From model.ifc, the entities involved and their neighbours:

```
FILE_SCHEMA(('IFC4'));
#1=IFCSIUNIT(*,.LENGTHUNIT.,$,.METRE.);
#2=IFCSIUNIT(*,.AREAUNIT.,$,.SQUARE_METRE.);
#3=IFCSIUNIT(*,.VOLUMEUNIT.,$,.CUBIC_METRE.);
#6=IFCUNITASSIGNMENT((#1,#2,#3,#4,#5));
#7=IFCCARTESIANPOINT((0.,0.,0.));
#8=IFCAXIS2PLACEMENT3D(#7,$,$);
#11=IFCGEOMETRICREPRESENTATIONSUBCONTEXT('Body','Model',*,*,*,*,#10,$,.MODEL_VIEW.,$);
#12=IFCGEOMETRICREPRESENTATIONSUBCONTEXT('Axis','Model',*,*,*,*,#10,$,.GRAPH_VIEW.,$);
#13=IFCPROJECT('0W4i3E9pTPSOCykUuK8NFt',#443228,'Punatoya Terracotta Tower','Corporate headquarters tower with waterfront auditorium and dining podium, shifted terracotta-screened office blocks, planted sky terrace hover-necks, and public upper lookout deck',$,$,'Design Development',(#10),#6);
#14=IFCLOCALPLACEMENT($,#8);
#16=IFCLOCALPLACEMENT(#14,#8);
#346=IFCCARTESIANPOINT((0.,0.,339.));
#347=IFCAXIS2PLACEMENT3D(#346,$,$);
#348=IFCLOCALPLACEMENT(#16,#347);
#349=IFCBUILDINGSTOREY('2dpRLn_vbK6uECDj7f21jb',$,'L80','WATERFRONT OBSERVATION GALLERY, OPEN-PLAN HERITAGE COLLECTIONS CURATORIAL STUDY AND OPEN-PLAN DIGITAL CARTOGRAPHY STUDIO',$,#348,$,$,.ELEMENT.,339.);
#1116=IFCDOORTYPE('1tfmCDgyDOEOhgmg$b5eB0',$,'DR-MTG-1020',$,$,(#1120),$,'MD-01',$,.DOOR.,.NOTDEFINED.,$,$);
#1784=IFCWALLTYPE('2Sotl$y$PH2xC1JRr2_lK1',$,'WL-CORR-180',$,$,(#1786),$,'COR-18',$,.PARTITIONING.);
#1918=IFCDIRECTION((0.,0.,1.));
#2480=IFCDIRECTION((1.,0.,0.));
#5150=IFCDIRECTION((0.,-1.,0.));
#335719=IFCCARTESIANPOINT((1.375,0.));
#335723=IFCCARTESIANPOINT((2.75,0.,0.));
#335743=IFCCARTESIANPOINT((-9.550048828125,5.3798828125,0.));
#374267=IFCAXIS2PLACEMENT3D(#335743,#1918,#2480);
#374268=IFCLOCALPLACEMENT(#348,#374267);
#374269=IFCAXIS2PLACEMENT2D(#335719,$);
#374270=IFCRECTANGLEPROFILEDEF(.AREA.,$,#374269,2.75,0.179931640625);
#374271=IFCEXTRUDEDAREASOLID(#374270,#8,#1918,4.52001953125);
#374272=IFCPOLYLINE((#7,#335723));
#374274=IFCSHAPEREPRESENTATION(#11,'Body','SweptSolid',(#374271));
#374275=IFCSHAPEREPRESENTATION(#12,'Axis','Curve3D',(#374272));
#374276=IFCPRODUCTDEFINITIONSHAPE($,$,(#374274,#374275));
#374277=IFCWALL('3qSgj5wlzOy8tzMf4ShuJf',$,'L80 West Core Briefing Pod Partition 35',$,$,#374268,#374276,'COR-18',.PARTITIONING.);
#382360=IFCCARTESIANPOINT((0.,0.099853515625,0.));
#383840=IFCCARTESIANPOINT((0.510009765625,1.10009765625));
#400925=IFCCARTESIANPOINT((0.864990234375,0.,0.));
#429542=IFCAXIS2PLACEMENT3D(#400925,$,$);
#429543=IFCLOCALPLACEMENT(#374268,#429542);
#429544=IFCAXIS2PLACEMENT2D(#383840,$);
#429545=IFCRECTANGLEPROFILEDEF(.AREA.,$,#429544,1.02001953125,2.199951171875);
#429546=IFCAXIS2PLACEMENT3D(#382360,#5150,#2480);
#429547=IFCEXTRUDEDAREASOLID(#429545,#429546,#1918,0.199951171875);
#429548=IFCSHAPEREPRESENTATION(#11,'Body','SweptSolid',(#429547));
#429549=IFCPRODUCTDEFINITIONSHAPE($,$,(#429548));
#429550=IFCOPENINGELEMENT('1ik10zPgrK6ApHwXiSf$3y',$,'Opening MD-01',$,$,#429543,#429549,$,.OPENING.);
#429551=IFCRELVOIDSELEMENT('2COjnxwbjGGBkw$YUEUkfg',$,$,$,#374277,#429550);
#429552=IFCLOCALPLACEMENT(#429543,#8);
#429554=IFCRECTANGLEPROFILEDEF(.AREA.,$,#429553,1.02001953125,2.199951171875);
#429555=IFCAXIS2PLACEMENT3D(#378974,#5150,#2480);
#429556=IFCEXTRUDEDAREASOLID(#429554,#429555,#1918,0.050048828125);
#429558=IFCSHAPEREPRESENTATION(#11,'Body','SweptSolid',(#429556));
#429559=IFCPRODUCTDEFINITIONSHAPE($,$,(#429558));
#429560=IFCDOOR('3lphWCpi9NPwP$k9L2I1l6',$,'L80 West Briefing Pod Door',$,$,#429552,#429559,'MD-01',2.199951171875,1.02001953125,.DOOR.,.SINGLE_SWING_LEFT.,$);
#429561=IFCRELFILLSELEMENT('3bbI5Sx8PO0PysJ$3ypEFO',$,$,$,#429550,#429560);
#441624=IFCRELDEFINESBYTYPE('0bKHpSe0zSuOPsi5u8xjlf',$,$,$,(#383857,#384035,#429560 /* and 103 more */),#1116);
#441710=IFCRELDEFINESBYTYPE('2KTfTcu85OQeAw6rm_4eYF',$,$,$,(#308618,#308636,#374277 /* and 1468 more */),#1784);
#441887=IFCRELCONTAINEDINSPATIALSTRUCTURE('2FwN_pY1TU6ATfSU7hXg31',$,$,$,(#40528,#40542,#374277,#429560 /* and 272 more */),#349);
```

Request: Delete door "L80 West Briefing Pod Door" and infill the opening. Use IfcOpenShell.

```python
import ifcopenshell
import ifcopenshell.api.feature
import ifcopenshell.api.root
import ifcopenshell.geom
import ifcopenshell.util.shape

model = ifcopenshell.open("model.ifc")
settings = ifcopenshell.geom.settings()


def volume(element):
    """Net volume in cubic metres, openings subtracted."""
    shape = ifcopenshell.geom.create_shape(settings, element)
    return ifcopenshell.util.shape.get_volume(shape.geometry)


door = model.by_guid("3lphWCpi9NPwP$k9L2I1l6")
opening = door.FillsVoids[0].RelatingOpeningElement
wall = opening.VoidsElements[0].RelatingBuildingElement
before = volume(wall)

ifcopenshell.api.root.remove_product(model, product=door)
ifcopenshell.api.feature.remove_feature(model, feature=opening)

after = volume(wall)

print(f"wall volume {before:.3f} -> {after:.3f} m3")

model.write("model_rev.ifc")
```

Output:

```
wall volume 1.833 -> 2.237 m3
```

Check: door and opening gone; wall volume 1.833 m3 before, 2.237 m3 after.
